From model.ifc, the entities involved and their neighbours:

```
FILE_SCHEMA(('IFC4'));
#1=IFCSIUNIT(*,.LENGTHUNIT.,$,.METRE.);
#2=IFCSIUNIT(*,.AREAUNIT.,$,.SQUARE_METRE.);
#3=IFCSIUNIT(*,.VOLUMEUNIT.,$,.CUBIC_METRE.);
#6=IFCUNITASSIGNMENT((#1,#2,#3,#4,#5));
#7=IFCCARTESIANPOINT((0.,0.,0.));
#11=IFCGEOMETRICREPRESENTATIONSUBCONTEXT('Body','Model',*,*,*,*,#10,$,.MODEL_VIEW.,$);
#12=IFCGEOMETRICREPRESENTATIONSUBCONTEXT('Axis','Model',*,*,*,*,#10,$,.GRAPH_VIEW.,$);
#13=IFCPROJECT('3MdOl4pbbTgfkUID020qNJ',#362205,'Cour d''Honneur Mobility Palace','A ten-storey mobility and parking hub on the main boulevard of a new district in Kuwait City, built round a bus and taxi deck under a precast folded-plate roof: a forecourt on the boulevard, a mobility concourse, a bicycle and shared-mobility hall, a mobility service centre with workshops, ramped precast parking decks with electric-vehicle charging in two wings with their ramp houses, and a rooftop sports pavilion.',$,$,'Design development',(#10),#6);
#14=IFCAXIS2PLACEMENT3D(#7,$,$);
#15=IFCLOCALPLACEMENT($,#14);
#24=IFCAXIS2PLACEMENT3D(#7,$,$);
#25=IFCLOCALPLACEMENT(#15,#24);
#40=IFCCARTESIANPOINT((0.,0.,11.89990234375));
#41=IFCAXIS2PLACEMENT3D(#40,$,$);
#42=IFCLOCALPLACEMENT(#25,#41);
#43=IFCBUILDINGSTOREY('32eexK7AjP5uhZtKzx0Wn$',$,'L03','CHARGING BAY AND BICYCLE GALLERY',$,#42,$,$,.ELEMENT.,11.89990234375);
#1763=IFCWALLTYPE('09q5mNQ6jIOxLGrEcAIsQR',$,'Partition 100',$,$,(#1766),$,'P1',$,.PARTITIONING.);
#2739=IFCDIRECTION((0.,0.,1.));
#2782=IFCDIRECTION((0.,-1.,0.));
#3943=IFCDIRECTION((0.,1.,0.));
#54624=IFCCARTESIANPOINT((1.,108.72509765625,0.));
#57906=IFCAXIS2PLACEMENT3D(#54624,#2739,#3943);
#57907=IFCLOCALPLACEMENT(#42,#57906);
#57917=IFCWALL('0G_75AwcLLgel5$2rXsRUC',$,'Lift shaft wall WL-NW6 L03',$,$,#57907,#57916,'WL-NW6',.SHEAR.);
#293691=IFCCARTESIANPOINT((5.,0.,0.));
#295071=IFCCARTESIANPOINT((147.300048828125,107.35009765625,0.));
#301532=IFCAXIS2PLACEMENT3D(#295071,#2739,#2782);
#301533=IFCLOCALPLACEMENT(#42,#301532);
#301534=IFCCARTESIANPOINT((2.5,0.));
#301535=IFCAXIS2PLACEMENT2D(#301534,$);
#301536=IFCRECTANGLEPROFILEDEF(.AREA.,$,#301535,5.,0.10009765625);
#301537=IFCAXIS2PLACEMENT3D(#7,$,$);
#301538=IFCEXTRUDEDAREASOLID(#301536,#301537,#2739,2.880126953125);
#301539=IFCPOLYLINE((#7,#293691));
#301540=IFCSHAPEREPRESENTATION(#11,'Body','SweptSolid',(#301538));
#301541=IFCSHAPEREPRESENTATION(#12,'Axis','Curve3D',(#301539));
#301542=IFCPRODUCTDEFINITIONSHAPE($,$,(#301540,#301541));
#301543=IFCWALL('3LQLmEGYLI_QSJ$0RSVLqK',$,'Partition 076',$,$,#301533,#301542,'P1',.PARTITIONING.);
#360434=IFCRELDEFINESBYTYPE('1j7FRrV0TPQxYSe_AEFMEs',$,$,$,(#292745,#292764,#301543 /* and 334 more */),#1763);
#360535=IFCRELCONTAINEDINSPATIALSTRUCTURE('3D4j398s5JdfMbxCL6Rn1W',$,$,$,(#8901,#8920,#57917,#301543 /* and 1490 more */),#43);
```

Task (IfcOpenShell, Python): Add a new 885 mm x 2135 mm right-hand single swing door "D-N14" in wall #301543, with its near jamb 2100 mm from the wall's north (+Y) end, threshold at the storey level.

```python
import numpy as np
import ifcopenshell
import ifcopenshell.api.feature
import ifcopenshell.api.geometry
import ifcopenshell.api.root
import ifcopenshell.api.spatial
import ifcopenshell.geom
import ifcopenshell.util.element
import ifcopenshell.util.placement
import ifcopenshell.util.representation
import ifcopenshell.util.shape
import ifcopenshell.util.unit

model = ifcopenshell.open("model.ifc")
unit_scale = ifcopenshell.util.unit.calculate_unit_scale(model)
settings = ifcopenshell.geom.settings()


def volume(element):
    """Net volume in cubic metres, openings subtracted."""
    shape = ifcopenshell.geom.create_shape(settings, element)
    return ifcopenshell.util.shape.get_volume(shape.geometry)


wall = model.by_guid("3LQLmEGYLI_QSJ$0RSVLqK")
storey = ifcopenshell.util.element.get_container(wall, ifc_class="IfcBuildingStorey")
context = ifcopenshell.util.representation.get_context(model, "Model", "Body", "MODEL_VIEW")
before = volume(wall)

width, height, from_end, sill = 0.885, 2.135, 2.1, 0.0  # metres

# The wall runs along its own X axis, and the end named is its -X end.
wall_shape = ifcopenshell.geom.create_shape(settings, wall)
x, y, z = ifcopenshell.util.shape.get_vertices(wall_shape.geometry).T
start = x.min() + from_end
face, thickness = float(y.min()), float(y.max() - y.min())
wall_matrix = ifcopenshell.util.placement.get_local_placement(wall.ObjectPlacement)
level = ifcopenshell.util.placement.get_local_placement(storey.ObjectPlacement)[2, 3]


def in_wall(x, y):
    """Placement at x, y metres in the wall's axes, at sill height."""
    matrix = wall_matrix.copy()
    matrix[:, 3] = wall_matrix @ np.array([x / unit_scale, y / unit_scale, 0.0, 1.0])
    matrix[2, 3] = level + sill / unit_scale
    return matrix


# Opening: a box that overshoots both wall faces by 50 mm.
opening = ifcopenshell.api.root.create_entity(model, ifc_class="IfcOpeningElement", predefined_type="OPENING")
box = ifcopenshell.api.geometry.add_wall_representation(
    model, context=context, length=width, height=height, thickness=thickness + 0.1
)
ifcopenshell.api.geometry.assign_representation(model, product=opening, representation=box)
ifcopenshell.api.geometry.edit_object_placement(model, product=opening, matrix=in_wall(start, face - 0.05), is_si=False)
ifcopenshell.api.feature.add_feature(model, feature=opening, element=wall)

door = ifcopenshell.api.root.create_entity(model, ifc_class="IfcDoor", name="D-N14", predefined_type="DOOR")
door.OverallWidth, door.OverallHeight = width / unit_scale, height / unit_scale
door.OperationType = "SINGLE_SWING_RIGHT"
body = ifcopenshell.api.geometry.add_door_representation(
    model,
    context=context,
    overall_width=door.OverallWidth,
    overall_height=door.OverallHeight,
    operation_type="SINGLE_SWING_RIGHT",
    lining_properties={"LiningDepth": thickness / unit_scale, "ThresholdDepth": thickness / unit_scale},
)
ifcopenshell.api.geometry.assign_representation(model, product=door, representation=body)
ifcopenshell.api.spatial.assign_container(model, products=[door], relating_structure=storey)
ifcopenshell.api.feature.add_filling(model, opening=opening, element=door)

# The lining spans the wall, so the door starts at the wall face.
ifcopenshell.api.geometry.edit_object_placement(model, product=door, matrix=in_wall(start, face), is_si=False)

after = volume(wall)

print(f"wall volume {before:.3f} -> {after:.3f} m3")

model.write("model_updated.ifc")
```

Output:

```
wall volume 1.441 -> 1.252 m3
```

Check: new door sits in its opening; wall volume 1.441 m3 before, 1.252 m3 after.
